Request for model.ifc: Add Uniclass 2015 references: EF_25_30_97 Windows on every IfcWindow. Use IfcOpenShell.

First a look at what the model holds.

```python
import ifcopenshell

model = ifcopenshell.open("model.ifc")
print(model.schema)
print("classifications:", [c.Name for c in model.by_type("IfcClassification")])
for ifc_class in ("IfcDoor", "IfcRoof", "IfcStair", "IfcWall", "IfcWindow"):
    print(ifc_class, len(model.by_type(ifc_class)))
```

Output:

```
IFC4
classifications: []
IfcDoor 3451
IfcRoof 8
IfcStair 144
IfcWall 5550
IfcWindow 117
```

```python
import ifcopenshell
import ifcopenshell.api.classification

model = ifcopenshell.open("model.ifc")

system = ifcopenshell.api.classification.add_classification(model, classification="Uniclass 2015")

codes = {
    "IfcWindow": ("EF_25_30_97", "Windows"),
}
for ifc_class, (code, name) in codes.items():
    products = model.by_type(ifc_class)
    ifcopenshell.api.classification.add_reference(
        model, products=products, classification=system, identification=code, name=name
    )
    print(code, len(products))

model.write("model-out.ifc")
```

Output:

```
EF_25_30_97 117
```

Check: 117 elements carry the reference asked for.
